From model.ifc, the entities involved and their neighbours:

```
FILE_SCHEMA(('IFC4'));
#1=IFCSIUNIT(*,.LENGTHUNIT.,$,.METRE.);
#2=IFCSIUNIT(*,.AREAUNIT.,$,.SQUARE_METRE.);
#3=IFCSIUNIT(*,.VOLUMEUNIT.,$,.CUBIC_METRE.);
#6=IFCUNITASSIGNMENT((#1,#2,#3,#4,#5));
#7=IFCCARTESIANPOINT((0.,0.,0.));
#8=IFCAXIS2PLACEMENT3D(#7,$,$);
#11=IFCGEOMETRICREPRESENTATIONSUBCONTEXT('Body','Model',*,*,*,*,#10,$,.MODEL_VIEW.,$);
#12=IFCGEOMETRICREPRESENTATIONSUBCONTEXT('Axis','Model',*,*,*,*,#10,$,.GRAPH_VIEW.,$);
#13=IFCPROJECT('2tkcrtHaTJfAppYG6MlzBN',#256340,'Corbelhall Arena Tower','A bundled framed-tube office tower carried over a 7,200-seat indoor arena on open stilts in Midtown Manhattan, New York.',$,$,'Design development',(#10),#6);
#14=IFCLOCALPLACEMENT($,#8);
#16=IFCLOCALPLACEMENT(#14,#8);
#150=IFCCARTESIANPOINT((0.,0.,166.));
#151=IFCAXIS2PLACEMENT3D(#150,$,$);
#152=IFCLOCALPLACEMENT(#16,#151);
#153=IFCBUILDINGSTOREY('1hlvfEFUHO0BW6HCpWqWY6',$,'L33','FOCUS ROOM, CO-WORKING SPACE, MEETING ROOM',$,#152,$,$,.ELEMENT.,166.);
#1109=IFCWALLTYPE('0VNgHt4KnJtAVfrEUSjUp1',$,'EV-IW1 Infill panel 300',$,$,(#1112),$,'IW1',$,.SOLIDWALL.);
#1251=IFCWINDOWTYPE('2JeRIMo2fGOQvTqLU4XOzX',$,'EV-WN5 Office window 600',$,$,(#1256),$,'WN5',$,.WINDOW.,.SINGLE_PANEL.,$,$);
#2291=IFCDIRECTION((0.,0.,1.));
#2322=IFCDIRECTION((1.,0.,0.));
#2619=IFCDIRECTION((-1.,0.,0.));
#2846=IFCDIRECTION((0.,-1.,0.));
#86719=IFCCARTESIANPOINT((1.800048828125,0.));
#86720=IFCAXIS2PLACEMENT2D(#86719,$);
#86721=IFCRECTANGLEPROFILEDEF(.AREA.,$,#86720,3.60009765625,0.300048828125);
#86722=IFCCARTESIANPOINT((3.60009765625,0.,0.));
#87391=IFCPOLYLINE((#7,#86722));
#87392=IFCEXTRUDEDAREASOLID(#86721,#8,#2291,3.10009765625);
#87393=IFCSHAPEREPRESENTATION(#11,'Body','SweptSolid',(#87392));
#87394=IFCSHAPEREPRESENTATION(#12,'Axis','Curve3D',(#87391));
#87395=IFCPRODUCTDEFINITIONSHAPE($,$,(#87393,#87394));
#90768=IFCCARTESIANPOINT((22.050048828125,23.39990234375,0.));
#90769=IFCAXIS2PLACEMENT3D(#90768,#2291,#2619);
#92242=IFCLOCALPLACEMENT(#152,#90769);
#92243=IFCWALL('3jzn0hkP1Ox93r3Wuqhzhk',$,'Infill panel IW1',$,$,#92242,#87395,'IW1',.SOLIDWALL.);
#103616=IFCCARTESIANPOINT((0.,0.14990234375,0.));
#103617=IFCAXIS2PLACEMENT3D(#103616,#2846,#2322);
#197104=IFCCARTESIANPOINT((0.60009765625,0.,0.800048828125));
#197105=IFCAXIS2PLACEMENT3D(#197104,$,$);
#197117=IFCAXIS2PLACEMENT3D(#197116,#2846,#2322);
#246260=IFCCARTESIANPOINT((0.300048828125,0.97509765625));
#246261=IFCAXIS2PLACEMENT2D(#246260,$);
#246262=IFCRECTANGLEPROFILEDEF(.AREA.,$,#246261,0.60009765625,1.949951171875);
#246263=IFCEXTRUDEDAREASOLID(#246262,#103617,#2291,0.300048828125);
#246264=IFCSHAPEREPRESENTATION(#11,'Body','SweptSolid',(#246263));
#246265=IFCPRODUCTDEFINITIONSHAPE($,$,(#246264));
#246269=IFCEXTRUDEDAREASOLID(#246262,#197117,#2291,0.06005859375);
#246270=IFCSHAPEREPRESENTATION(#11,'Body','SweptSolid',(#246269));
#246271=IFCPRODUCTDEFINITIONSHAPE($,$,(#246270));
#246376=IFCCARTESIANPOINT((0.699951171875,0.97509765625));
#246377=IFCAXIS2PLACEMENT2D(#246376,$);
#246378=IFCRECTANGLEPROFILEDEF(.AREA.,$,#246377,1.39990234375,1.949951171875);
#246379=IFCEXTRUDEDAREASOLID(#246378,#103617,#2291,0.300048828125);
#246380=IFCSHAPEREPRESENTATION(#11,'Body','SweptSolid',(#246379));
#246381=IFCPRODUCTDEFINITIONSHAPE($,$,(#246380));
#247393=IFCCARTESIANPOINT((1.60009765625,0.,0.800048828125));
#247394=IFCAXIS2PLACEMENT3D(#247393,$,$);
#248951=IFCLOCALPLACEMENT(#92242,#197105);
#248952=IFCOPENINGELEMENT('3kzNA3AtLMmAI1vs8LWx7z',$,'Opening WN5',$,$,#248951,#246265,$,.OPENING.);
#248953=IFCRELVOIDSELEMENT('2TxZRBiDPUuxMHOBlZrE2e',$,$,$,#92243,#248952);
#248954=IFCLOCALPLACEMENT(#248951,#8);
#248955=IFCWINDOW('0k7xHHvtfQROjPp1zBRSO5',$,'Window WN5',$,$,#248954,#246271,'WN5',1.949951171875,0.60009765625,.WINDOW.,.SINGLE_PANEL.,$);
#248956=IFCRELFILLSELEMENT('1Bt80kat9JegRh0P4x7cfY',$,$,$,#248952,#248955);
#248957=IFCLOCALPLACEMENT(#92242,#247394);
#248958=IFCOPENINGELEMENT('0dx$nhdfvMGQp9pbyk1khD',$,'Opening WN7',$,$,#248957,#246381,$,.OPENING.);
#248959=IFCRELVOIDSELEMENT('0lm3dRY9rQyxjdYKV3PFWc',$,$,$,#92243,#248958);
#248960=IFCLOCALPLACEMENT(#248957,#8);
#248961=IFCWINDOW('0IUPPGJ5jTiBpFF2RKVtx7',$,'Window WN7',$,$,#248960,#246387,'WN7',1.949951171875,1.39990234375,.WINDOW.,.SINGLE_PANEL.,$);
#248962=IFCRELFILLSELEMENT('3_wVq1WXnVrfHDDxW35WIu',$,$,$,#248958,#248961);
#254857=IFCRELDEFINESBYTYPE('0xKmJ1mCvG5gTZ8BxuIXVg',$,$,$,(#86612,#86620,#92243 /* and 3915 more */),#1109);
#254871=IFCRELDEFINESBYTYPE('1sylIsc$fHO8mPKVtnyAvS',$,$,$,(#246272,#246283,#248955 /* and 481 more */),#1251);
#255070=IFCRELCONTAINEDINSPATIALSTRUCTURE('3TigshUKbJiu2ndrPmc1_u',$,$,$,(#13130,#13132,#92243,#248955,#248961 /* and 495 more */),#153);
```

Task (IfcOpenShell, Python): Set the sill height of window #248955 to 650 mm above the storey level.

```python
import numpy as np
import ifcopenshell
import ifcopenshell.api.geometry
import ifcopenshell.geom
import ifcopenshell.util.element
import ifcopenshell.util.placement
import ifcopenshell.util.shape
import ifcopenshell.util.unit

model = ifcopenshell.open("model.ifc")
unit_scale = ifcopenshell.util.unit.calculate_unit_scale(model)

window = model.by_guid("0k7xHHvtfQROjPp1zBRSO5")
opening = window.FillsVoids[0].RelatingOpeningElement
storey = ifcopenshell.util.element.get_container(window, ifc_class="IfcBuildingStorey")
level = ifcopenshell.util.placement.get_local_placement(storey.ObjectPlacement)[2, 3]

# The opening's origin need not be at the sill, so measure its lowest point.
shape = ifcopenshell.geom.create_shape(ifcopenshell.geom.settings(), opening)
bottom = ifcopenshell.util.shape.get_shape_bottom_elevation(shape, shape.geometry) / unit_scale
dz = level + 0.65 / unit_scale - bottom

shift = np.array([0.0, 0.0, dz])
# The window is placed relative to its opening, so it follows when the opening moves.
matrix = ifcopenshell.util.placement.get_local_placement(opening.ObjectPlacement)
matrix[:3, 3] += shift
ifcopenshell.api.geometry.edit_object_placement(
    model, product=opening, matrix=matrix, is_si=False, should_transform_children=True
)

print(f"moved by {dz * unit_scale:+.3f} m")

model.write("model_edited.ifc")
```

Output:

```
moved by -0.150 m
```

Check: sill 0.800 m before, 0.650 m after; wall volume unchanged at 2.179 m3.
